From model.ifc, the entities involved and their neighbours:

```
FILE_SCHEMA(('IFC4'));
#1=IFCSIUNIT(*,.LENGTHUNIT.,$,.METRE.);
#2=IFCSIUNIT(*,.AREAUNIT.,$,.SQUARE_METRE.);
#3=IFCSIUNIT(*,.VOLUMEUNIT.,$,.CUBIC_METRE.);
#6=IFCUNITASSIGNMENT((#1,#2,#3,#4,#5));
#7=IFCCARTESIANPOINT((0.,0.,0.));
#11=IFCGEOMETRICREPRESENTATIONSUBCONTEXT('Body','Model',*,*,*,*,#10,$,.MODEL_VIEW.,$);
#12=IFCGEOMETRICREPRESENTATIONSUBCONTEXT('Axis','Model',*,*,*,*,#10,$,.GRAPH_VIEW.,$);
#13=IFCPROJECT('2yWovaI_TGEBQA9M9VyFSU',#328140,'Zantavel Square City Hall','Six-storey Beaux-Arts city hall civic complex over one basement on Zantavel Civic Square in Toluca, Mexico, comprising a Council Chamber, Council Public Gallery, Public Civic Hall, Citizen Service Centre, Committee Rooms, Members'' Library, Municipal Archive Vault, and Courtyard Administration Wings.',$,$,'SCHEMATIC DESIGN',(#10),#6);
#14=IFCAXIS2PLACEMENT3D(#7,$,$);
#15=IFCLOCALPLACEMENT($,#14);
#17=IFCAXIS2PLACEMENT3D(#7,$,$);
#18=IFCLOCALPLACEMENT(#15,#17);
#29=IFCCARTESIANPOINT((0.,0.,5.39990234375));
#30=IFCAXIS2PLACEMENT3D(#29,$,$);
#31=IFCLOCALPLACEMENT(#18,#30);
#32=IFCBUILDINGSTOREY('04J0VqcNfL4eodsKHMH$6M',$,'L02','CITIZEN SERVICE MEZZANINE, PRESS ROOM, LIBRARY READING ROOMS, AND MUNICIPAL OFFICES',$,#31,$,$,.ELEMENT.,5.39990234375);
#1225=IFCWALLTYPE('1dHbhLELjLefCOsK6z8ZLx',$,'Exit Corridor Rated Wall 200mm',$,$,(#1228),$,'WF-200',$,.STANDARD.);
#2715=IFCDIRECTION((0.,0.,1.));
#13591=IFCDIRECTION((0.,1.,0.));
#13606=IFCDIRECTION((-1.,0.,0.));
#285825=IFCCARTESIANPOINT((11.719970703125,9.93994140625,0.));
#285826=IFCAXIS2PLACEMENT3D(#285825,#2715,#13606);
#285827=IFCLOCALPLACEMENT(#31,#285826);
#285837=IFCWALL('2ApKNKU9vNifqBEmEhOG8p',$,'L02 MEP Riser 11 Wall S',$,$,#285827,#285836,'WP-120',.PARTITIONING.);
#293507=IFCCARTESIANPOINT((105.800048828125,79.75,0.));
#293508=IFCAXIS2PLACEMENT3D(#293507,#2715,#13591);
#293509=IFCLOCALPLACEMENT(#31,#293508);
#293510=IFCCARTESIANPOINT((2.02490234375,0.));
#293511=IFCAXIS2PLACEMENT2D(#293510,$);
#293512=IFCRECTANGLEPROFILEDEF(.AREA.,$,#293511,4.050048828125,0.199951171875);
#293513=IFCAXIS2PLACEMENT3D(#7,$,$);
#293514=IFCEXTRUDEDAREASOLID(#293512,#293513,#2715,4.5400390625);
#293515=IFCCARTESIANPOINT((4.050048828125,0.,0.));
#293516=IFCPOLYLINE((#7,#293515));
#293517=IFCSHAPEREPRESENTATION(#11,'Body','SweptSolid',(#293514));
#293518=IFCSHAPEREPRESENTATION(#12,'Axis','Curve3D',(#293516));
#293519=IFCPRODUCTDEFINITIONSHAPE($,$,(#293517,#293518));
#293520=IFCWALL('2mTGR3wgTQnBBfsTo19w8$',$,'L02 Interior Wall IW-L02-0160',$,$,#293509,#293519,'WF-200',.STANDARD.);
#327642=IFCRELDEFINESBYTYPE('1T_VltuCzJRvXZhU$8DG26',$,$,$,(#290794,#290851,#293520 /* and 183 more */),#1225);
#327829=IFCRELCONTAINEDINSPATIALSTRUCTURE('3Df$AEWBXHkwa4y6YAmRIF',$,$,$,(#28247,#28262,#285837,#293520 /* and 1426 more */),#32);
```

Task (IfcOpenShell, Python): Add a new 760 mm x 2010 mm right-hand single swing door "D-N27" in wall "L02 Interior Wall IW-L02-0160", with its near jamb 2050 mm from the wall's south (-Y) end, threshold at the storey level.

```python
import numpy as np
import ifcopenshell
import ifcopenshell.api.feature
import ifcopenshell.api.geometry
import ifcopenshell.api.root
import ifcopenshell.api.spatial
import ifcopenshell.geom
import ifcopenshell.util.element
import ifcopenshell.util.placement
import ifcopenshell.util.representation
import ifcopenshell.util.shape
import ifcopenshell.util.unit

model = ifcopenshell.open("model.ifc")
unit_scale = ifcopenshell.util.unit.calculate_unit_scale(model)
settings = ifcopenshell.geom.settings()


def volume(element):
    """Net volume in cubic metres, openings subtracted."""
    shape = ifcopenshell.geom.create_shape(settings, element)
    return ifcopenshell.util.shape.get_volume(shape.geometry)


wall = model.by_id(293520)
storey = ifcopenshell.util.element.get_container(wall, ifc_class="IfcBuildingStorey")
context = ifcopenshell.util.representation.get_context(model, "Model", "Body", "MODEL_VIEW")
before = volume(wall)

width, height, from_end, sill = 0.76, 2.01, 2.05, 0.0  # metres

# The wall runs along its own X axis, and the end named is its -X end.
wall_shape = ifcopenshell.geom.create_shape(settings, wall)
x, y, z = ifcopenshell.util.shape.get_vertices(wall_shape.geometry).T
start = x.min() + from_end
face, thickness = float(y.min()), float(y.max() - y.min())
wall_matrix = ifcopenshell.util.placement.get_local_placement(wall.ObjectPlacement)
level = ifcopenshell.util.placement.get_local_placement(storey.ObjectPlacement)[2, 3]


def in_wall(x, y):
    """Placement at x, y metres in the wall's axes, at sill height."""
    matrix = wall_matrix.copy()
    matrix[:, 3] = wall_matrix @ np.array([x / unit_scale, y / unit_scale, 0.0, 1.0])
    matrix[2, 3] = level + sill / unit_scale
    return matrix


# Opening: a box that overshoots both wall faces by 50 mm.
opening = ifcopenshell.api.root.create_entity(model, ifc_class="IfcOpeningElement", predefined_type="OPENING")
box = ifcopenshell.api.geometry.add_wall_representation(
    model, context=context, length=width, height=height, thickness=thickness + 0.1
)
ifcopenshell.api.geometry.assign_representation(model, product=opening, representation=box)
ifcopenshell.api.geometry.edit_object_placement(model, product=opening, matrix=in_wall(start, face - 0.05), is_si=False)
ifcopenshell.api.feature.add_feature(model, feature=opening, element=wall)

door = ifcopenshell.api.root.create_entity(model, ifc_class="IfcDoor", name="D-N27", predefined_type="DOOR")
door.OverallWidth, door.OverallHeight = width / unit_scale, height / unit_scale
door.OperationType = "SINGLE_SWING_RIGHT"
body = ifcopenshell.api.geometry.add_door_representation(
    model,
    context=context,
    overall_width=door.OverallWidth,
    overall_height=door.OverallHeight,
    operation_type="SINGLE_SWING_RIGHT",
    lining_properties={"LiningDepth": thickness / unit_scale, "ThresholdDepth": thickness / unit_scale},
)
ifcopenshell.api.geometry.assign_representation(model, product=door, representation=body)
ifcopenshell.api.spatial.assign_container(model, products=[door], relating_structure=storey)
ifcopenshell.api.feature.add_filling(model, opening=opening, element=door)

# The lining spans the wall, so the door starts at the wall face.
ifcopenshell.api.geometry.edit_object_placement(model, product=door, matrix=in_wall(start, face), is_si=False)

after = volume(wall)

print(f"wall volume {before:.3f} -> {after:.3f} m3")

model.write("model-out.ifc")
```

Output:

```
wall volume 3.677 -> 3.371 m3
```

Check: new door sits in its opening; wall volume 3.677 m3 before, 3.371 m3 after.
